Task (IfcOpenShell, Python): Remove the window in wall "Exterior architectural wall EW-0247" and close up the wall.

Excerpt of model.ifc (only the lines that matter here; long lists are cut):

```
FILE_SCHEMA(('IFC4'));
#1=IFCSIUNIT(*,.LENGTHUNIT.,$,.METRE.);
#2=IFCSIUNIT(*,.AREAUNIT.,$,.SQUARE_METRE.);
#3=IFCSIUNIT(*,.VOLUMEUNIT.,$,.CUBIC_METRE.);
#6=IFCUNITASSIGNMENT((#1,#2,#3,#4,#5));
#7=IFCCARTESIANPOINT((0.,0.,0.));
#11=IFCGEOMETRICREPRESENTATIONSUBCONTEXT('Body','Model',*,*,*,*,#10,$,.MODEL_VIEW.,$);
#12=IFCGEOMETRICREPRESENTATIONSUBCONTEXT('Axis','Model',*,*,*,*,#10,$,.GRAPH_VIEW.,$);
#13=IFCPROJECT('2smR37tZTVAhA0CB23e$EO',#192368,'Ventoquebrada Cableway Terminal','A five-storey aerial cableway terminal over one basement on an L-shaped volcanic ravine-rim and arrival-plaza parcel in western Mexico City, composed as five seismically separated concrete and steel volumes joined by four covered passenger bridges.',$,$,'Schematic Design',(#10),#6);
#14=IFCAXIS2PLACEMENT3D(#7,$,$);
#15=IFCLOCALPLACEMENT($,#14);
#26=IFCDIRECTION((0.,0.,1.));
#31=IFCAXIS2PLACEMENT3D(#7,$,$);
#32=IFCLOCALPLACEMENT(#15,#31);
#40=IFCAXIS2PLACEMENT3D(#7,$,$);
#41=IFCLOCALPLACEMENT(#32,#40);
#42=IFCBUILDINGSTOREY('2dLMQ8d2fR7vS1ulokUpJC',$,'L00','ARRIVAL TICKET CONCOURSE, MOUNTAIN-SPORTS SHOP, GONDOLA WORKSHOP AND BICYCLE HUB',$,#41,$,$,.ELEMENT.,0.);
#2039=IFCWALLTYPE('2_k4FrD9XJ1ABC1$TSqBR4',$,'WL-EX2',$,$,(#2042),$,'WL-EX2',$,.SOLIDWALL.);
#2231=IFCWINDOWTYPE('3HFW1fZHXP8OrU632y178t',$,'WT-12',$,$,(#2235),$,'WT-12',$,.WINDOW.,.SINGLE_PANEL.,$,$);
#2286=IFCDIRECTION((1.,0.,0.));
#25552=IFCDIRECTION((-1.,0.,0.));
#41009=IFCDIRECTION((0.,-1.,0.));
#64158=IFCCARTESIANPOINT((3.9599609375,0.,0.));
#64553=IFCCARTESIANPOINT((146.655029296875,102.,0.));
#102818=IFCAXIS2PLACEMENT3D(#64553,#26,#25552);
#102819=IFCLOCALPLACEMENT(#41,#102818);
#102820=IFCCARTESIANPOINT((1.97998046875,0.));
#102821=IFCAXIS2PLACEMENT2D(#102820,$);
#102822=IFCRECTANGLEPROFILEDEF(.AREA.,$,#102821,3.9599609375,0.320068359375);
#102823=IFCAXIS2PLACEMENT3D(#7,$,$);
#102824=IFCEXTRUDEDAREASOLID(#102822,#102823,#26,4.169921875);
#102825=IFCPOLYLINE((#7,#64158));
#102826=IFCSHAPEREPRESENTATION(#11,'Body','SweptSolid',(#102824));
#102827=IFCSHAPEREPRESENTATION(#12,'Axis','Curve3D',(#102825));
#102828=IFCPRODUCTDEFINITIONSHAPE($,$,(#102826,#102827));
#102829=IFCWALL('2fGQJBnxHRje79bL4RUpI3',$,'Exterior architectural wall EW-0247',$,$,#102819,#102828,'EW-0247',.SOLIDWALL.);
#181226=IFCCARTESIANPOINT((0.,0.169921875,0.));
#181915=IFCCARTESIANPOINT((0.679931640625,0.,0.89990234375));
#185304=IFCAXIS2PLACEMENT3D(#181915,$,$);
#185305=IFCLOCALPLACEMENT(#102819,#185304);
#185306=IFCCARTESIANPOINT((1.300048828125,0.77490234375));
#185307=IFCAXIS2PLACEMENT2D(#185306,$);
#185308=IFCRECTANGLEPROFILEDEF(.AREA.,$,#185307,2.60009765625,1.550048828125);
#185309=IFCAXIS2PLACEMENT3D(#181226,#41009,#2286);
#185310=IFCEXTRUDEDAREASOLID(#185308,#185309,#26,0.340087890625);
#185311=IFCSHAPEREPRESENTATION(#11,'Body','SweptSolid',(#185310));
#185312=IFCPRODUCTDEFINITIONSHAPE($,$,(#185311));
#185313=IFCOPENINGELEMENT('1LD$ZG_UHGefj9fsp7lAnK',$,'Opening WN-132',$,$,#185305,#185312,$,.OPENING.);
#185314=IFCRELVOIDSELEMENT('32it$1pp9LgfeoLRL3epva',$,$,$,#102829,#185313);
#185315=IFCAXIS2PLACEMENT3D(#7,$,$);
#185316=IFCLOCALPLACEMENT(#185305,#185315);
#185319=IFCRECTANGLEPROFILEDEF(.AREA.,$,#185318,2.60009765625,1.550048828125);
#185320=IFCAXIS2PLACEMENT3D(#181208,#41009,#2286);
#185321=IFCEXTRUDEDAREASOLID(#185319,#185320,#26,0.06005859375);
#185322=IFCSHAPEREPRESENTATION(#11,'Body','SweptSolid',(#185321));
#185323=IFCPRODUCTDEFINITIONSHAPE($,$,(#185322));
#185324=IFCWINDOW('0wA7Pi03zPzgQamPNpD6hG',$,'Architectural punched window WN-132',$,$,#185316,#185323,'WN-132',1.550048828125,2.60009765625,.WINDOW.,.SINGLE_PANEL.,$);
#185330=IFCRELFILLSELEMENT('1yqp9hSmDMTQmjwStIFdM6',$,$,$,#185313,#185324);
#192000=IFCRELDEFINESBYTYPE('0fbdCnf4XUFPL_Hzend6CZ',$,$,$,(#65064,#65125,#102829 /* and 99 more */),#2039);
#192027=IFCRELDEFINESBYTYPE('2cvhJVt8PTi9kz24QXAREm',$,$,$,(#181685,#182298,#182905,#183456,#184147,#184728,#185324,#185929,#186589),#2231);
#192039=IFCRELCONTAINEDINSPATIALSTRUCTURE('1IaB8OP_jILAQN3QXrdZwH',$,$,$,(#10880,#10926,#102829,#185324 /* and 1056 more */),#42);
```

```python
import ifcopenshell
import ifcopenshell.api.feature
import ifcopenshell.api.root
import ifcopenshell.geom
import ifcopenshell.util.shape

model = ifcopenshell.open("model.ifc")
settings = ifcopenshell.geom.settings()


def volume(element):
    """Net volume in cubic metres, openings subtracted."""
    shape = ifcopenshell.geom.create_shape(settings, element)
    return ifcopenshell.util.shape.get_volume(shape.geometry)


window = model.by_guid("0wA7Pi03zPzgQamPNpD6hG")
opening = window.FillsVoids[0].RelatingOpeningElement
wall = opening.VoidsElements[0].RelatingBuildingElement
before = volume(wall)

ifcopenshell.api.root.remove_product(model, product=window)
ifcopenshell.api.feature.remove_feature(model, feature=opening)

after = volume(wall)

print(f"wall volume {before:.3f} -> {after:.3f} m3")

model.write("model-out.ifc")
```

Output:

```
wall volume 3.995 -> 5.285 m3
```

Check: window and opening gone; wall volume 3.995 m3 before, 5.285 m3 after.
